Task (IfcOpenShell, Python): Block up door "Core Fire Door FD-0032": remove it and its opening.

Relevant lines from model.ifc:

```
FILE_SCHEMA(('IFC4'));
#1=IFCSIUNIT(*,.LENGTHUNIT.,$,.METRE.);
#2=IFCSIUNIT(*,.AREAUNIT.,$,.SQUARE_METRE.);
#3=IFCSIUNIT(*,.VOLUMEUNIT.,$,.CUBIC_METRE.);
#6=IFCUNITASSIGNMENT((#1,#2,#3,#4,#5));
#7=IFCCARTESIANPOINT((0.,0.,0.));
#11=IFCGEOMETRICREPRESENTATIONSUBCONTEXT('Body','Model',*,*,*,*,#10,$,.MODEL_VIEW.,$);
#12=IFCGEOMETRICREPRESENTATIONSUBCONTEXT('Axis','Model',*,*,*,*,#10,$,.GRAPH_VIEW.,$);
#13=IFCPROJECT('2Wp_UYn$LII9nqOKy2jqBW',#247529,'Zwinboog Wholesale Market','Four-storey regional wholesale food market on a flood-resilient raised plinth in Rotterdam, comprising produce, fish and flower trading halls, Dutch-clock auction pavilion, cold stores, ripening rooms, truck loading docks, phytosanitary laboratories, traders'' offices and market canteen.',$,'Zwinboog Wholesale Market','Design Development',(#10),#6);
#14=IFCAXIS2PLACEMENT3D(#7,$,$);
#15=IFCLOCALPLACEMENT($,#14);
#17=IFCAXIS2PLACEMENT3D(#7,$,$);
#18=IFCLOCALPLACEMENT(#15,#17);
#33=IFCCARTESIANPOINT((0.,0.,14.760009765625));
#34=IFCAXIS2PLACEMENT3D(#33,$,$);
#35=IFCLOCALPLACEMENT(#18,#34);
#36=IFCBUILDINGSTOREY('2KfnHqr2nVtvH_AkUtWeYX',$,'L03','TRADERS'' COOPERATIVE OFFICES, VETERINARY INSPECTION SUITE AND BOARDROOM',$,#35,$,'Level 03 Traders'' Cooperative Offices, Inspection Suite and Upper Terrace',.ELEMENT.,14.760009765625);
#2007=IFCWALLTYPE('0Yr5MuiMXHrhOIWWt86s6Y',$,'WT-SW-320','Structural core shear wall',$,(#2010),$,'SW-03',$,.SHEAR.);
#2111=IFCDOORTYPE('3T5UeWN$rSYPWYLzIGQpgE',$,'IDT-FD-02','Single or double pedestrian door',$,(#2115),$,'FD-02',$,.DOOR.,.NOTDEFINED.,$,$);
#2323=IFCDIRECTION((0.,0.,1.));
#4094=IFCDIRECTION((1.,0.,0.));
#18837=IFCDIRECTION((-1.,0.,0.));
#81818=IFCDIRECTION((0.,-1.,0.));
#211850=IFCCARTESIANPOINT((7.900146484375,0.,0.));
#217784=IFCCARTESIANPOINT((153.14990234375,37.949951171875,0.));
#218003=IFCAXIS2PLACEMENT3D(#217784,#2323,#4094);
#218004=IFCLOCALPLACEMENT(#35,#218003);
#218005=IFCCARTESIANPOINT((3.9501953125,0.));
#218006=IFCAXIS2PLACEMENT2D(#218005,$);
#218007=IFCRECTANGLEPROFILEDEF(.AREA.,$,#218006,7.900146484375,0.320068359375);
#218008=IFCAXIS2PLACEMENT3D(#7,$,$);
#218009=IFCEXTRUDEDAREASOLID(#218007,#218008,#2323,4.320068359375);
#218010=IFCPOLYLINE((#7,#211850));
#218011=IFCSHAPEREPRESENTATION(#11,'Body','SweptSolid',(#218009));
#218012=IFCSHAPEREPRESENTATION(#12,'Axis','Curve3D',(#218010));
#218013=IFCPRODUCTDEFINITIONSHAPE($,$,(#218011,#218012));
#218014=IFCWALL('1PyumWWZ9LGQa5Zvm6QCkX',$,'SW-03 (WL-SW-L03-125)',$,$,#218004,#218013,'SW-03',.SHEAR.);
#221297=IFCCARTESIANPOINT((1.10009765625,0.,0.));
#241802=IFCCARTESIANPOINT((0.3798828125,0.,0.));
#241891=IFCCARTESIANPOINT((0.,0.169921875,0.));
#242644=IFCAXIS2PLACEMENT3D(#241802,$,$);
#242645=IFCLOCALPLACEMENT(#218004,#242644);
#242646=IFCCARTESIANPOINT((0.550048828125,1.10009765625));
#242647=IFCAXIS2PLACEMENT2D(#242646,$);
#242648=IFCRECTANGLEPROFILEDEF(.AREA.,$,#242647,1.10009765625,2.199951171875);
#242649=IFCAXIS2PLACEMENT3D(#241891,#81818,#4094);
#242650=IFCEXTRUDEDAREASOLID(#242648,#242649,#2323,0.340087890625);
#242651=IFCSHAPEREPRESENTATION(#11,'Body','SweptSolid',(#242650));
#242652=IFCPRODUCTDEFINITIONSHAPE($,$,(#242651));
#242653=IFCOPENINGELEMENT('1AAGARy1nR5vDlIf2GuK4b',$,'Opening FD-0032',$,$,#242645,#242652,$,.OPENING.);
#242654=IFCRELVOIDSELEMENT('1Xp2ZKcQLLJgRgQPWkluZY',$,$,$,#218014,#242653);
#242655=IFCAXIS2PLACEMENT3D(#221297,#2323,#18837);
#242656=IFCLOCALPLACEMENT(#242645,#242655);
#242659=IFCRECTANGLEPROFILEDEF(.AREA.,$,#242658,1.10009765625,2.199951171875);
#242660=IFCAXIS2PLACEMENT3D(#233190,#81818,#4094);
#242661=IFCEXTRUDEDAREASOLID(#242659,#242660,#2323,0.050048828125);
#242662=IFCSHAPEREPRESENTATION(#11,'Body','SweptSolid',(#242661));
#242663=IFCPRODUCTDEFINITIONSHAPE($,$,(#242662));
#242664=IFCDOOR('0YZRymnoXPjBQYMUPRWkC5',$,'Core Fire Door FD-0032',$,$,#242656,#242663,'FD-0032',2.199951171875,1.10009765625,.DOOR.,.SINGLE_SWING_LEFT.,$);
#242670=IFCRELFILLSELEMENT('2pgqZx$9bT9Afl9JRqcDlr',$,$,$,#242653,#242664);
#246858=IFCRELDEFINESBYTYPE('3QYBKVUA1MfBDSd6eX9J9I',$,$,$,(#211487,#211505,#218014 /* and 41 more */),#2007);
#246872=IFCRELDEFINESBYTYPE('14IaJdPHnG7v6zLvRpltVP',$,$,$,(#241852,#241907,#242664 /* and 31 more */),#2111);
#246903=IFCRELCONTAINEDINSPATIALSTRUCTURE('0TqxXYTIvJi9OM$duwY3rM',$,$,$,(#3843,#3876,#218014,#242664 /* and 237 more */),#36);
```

```python
import ifcopenshell
import ifcopenshell.api.feature
import ifcopenshell.api.root
import ifcopenshell.geom
import ifcopenshell.util.shape

model = ifcopenshell.open("model.ifc")
settings = ifcopenshell.geom.settings()


def volume(element):
    """Net volume in cubic metres, openings subtracted."""
    shape = ifcopenshell.geom.create_shape(settings, element)
    return ifcopenshell.util.shape.get_volume(shape.geometry)


door = model.by_id(242664)
opening = door.FillsVoids[0].RelatingOpeningElement
wall = opening.VoidsElements[0].RelatingBuildingElement
before = volume(wall)

ifcopenshell.api.root.remove_product(model, product=door)
ifcopenshell.api.feature.remove_feature(model, feature=opening)

after = volume(wall)

print(f"wall volume {before:.3f} -> {after:.3f} m3")

model.write("model_edited.ifc")
```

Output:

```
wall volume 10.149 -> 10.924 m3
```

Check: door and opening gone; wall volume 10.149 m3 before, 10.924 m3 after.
